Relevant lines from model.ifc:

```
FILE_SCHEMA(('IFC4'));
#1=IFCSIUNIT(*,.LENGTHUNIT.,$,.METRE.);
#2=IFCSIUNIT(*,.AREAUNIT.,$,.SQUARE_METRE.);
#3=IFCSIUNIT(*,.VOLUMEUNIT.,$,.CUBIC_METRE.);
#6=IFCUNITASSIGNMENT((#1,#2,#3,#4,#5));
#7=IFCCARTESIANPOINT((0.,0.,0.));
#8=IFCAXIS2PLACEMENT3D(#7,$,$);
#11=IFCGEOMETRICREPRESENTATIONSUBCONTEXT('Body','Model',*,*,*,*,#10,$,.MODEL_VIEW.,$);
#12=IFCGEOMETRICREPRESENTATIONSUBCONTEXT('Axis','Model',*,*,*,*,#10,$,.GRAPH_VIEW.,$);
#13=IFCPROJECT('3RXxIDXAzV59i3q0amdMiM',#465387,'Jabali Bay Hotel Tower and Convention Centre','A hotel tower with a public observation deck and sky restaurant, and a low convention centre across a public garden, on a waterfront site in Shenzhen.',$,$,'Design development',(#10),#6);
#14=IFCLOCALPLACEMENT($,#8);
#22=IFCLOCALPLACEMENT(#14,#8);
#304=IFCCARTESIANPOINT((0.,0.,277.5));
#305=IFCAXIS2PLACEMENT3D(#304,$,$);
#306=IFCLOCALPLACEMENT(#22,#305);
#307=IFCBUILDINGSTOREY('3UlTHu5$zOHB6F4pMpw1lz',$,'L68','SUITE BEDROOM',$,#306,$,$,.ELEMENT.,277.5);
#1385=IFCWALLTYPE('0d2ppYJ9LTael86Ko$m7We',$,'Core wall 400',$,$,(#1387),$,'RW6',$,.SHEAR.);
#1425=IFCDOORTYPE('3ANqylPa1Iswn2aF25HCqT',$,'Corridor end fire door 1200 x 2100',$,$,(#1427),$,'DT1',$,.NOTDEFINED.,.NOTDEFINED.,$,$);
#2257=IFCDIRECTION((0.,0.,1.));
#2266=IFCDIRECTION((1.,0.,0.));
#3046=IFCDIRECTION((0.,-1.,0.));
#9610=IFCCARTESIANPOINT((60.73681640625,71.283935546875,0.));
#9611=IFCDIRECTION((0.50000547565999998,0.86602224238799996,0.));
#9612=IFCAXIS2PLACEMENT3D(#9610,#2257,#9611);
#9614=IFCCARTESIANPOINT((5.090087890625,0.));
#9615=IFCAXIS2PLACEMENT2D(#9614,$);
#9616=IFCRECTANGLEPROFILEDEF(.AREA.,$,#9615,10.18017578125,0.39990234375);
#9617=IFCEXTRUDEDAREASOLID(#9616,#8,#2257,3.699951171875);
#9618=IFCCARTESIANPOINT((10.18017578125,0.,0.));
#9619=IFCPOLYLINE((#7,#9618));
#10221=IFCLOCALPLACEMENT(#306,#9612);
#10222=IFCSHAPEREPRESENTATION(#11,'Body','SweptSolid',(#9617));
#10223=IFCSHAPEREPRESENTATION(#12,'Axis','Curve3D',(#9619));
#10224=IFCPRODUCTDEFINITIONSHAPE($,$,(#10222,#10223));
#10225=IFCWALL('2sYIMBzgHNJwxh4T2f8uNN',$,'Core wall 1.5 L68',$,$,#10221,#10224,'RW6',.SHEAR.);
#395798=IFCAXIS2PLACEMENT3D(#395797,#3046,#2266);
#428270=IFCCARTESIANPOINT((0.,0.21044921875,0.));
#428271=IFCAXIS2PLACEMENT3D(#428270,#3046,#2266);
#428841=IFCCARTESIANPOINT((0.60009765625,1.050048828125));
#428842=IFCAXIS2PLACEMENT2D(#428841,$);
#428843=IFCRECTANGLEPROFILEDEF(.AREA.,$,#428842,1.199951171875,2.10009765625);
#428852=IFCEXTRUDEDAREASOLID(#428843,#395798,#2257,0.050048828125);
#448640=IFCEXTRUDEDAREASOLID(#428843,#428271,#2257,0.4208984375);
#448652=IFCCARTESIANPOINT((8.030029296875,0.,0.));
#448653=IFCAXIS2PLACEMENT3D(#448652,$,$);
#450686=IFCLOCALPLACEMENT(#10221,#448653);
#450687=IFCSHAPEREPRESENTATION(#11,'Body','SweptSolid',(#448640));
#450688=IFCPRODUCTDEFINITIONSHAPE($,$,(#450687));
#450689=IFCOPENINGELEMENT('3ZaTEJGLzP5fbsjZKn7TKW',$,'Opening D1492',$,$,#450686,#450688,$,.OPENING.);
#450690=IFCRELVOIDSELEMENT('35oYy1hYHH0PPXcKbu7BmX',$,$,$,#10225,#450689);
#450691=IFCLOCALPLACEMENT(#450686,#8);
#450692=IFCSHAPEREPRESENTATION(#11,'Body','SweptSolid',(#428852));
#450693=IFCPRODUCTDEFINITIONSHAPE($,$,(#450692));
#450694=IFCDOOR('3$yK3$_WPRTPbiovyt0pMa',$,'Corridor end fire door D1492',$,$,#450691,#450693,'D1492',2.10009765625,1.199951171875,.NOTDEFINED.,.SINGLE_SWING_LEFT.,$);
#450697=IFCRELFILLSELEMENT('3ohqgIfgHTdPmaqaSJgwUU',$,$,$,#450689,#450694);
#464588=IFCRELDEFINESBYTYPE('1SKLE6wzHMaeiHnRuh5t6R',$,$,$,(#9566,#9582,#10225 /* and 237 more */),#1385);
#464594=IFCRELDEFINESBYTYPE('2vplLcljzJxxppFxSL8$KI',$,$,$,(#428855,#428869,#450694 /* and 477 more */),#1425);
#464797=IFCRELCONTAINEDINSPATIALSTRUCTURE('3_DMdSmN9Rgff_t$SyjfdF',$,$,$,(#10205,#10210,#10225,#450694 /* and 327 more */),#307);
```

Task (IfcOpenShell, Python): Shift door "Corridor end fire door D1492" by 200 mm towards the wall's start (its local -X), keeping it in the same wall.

```python
import ifcopenshell
import ifcopenshell.api.geometry
import ifcopenshell.util.placement

model = ifcopenshell.open("model.ifc")

door = model.by_id(450694)
opening = door.FillsVoids[0].RelatingOpeningElement
wall = opening.VoidsElements[0].RelatingBuildingElement

wall_matrix = ifcopenshell.util.placement.get_local_placement(wall.ObjectPlacement)
shift = wall_matrix[:3, 0] * -0.2
before = ifcopenshell.util.placement.get_local_placement(door.ObjectPlacement)[:3, 3].copy()

# The door is placed relative to its opening, so it follows when the opening moves.
matrix = ifcopenshell.util.placement.get_local_placement(opening.ObjectPlacement)
matrix[:3, 3] += shift
ifcopenshell.api.geometry.edit_object_placement(
    model, product=opening, matrix=matrix, is_si=False, should_transform_children=True
)

after = ifcopenshell.util.placement.get_local_placement(door.ObjectPlacement)[:3, 3]
print("door moved by", (after - before).round(3) + 0.0)

model.write("model_edited.ifc")
```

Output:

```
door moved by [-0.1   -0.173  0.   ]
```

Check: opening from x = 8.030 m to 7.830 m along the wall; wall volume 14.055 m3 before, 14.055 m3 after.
